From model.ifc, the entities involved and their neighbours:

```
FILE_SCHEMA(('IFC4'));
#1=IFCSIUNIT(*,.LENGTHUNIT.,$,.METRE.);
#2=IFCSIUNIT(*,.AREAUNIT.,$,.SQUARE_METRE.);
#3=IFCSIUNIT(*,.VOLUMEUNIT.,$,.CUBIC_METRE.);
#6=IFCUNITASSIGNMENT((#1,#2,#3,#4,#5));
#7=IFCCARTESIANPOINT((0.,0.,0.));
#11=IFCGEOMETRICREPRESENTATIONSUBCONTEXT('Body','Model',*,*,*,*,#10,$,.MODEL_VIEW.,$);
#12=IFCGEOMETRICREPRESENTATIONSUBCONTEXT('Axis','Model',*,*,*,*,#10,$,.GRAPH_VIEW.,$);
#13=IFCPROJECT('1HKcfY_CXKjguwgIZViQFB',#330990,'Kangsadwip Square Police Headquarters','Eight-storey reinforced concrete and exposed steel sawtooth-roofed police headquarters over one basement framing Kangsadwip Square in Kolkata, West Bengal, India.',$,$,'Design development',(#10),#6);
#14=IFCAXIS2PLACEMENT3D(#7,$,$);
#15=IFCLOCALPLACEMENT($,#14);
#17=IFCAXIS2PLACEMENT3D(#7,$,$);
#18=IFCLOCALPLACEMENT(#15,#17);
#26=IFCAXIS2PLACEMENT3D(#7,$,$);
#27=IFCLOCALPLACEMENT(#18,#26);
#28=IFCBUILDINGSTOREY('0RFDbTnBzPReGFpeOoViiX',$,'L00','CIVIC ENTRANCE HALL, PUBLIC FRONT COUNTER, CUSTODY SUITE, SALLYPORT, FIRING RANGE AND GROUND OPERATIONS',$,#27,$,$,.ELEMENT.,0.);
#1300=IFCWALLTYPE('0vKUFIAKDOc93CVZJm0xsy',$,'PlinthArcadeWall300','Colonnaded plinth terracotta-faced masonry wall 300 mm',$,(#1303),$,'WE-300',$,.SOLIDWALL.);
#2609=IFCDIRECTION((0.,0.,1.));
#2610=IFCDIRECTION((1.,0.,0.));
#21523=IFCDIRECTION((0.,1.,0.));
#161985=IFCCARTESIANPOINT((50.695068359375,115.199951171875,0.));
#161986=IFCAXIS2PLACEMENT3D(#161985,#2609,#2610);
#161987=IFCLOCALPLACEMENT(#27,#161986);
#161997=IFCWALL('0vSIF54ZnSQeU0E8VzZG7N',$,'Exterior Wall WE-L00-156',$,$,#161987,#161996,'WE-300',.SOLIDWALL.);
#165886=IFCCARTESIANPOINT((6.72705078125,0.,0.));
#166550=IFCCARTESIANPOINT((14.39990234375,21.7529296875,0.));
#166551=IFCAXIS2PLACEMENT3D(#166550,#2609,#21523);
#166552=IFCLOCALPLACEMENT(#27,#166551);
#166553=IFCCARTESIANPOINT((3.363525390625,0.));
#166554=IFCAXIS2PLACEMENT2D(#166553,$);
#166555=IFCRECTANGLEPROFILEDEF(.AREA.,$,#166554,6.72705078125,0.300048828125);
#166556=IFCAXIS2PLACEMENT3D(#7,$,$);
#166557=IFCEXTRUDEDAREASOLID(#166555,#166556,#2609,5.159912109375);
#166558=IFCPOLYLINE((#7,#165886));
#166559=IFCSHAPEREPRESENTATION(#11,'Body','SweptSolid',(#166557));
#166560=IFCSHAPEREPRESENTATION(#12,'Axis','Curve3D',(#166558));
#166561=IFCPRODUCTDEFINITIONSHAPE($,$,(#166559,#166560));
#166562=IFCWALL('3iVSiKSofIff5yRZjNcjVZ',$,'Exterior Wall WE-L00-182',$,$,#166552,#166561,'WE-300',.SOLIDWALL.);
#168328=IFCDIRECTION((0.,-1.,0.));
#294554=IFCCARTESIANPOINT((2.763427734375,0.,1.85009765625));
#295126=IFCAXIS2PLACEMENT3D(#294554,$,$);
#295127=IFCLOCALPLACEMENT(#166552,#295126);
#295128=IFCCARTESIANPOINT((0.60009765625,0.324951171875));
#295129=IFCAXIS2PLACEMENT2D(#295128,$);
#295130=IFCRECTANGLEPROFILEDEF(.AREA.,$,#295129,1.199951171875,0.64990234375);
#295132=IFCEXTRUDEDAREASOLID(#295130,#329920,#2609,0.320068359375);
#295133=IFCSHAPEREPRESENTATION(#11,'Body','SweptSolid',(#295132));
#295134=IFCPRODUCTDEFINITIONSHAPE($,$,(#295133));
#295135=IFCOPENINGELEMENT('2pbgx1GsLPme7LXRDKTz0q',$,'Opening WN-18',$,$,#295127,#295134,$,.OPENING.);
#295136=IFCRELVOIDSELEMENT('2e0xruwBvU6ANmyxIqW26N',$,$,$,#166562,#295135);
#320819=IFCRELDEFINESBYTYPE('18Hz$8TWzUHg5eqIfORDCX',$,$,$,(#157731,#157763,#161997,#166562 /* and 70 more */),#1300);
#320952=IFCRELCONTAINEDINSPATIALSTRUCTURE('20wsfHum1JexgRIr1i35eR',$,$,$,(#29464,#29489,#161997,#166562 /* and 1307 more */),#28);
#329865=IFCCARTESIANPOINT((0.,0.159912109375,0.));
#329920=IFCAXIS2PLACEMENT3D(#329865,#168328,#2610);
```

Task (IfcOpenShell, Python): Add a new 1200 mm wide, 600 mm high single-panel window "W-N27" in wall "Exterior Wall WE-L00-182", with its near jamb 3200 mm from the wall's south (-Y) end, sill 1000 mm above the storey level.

```python
import numpy as np
import ifcopenshell
import ifcopenshell.api.feature
import ifcopenshell.api.geometry
import ifcopenshell.api.root
import ifcopenshell.api.spatial
import ifcopenshell.geom
import ifcopenshell.util.element
import ifcopenshell.util.placement
import ifcopenshell.util.representation
import ifcopenshell.util.shape
import ifcopenshell.util.unit

model = ifcopenshell.open("model.ifc")
unit_scale = ifcopenshell.util.unit.calculate_unit_scale(model)
settings = ifcopenshell.geom.settings()


def volume(element):
    """Net volume in cubic metres, openings subtracted."""
    shape = ifcopenshell.geom.create_shape(settings, element)
    return ifcopenshell.util.shape.get_volume(shape.geometry)


wall = model.by_guid("3iVSiKSofIff5yRZjNcjVZ")
storey = ifcopenshell.util.element.get_container(wall, ifc_class="IfcBuildingStorey")
context = ifcopenshell.util.representation.get_context(model, "Model", "Body", "MODEL_VIEW")
before = volume(wall)

width, height, from_end, sill = 1.2, 0.6, 3.2, 1  # metres

# The wall runs along its own X axis, and the end named is its -X end.
wall_shape = ifcopenshell.geom.create_shape(settings, wall)
x, y, z = ifcopenshell.util.shape.get_vertices(wall_shape.geometry).T
start = x.min() + from_end
face, thickness = float(y.min()), float(y.max() - y.min())
wall_matrix = ifcopenshell.util.placement.get_local_placement(wall.ObjectPlacement)
level = ifcopenshell.util.placement.get_local_placement(storey.ObjectPlacement)[2, 3]


def in_wall(x, y):
    """Placement at x, y metres in the wall's axes, at sill height."""
    matrix = wall_matrix.copy()
    matrix[:, 3] = wall_matrix @ np.array([x / unit_scale, y / unit_scale, 0.0, 1.0])
    matrix[2, 3] = level + sill / unit_scale
    return matrix


# Opening: a box that overshoots both wall faces by 50 mm.
opening = ifcopenshell.api.root.create_entity(model, ifc_class="IfcOpeningElement", predefined_type="OPENING")
box = ifcopenshell.api.geometry.add_wall_representation(
    model, context=context, length=width, height=height, thickness=thickness + 0.1
)
ifcopenshell.api.geometry.assign_representation(model, product=opening, representation=box)
ifcopenshell.api.geometry.edit_object_placement(model, product=opening, matrix=in_wall(start, face - 0.05), is_si=False)
ifcopenshell.api.feature.add_feature(model, feature=opening, element=wall)

window = ifcopenshell.api.root.create_entity(model, ifc_class="IfcWindow", name="W-N27", predefined_type="WINDOW")
window.OverallWidth, window.OverallHeight = width / unit_scale, height / unit_scale
window.PartitioningType = "SINGLE_PANEL"
body = ifcopenshell.api.geometry.add_window_representation(
    model,
    context=context,
    overall_width=window.OverallWidth,
    overall_height=window.OverallHeight,
    partition_type="SINGLE_PANEL",
)
ifcopenshell.api.geometry.assign_representation(model, product=window, representation=body)
ifcopenshell.api.spatial.assign_container(model, products=[window], relating_structure=storey)
ifcopenshell.api.feature.add_filling(model, opening=opening, element=window)

# Centre the window in the wall's thickness.
ifcopenshell.api.geometry.edit_object_placement(model, product=window, matrix=in_wall(start, face), is_si=False)
window_shape = ifcopenshell.geom.create_shape(settings, window)
depth = ifcopenshell.util.shape.get_vertices(window_shape.geometry)[:, 1]
offset = face + thickness / 2 - (depth.min() + depth.max()) / 2
ifcopenshell.api.geometry.edit_object_placement(model, product=window, matrix=in_wall(start, offset), is_si=False)

after = volume(wall)

print(f"wall volume {before:.3f} -> {after:.3f} m3")

model.write("model-out.ifc")
```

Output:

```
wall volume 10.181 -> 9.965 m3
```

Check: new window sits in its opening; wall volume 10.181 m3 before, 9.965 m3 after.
